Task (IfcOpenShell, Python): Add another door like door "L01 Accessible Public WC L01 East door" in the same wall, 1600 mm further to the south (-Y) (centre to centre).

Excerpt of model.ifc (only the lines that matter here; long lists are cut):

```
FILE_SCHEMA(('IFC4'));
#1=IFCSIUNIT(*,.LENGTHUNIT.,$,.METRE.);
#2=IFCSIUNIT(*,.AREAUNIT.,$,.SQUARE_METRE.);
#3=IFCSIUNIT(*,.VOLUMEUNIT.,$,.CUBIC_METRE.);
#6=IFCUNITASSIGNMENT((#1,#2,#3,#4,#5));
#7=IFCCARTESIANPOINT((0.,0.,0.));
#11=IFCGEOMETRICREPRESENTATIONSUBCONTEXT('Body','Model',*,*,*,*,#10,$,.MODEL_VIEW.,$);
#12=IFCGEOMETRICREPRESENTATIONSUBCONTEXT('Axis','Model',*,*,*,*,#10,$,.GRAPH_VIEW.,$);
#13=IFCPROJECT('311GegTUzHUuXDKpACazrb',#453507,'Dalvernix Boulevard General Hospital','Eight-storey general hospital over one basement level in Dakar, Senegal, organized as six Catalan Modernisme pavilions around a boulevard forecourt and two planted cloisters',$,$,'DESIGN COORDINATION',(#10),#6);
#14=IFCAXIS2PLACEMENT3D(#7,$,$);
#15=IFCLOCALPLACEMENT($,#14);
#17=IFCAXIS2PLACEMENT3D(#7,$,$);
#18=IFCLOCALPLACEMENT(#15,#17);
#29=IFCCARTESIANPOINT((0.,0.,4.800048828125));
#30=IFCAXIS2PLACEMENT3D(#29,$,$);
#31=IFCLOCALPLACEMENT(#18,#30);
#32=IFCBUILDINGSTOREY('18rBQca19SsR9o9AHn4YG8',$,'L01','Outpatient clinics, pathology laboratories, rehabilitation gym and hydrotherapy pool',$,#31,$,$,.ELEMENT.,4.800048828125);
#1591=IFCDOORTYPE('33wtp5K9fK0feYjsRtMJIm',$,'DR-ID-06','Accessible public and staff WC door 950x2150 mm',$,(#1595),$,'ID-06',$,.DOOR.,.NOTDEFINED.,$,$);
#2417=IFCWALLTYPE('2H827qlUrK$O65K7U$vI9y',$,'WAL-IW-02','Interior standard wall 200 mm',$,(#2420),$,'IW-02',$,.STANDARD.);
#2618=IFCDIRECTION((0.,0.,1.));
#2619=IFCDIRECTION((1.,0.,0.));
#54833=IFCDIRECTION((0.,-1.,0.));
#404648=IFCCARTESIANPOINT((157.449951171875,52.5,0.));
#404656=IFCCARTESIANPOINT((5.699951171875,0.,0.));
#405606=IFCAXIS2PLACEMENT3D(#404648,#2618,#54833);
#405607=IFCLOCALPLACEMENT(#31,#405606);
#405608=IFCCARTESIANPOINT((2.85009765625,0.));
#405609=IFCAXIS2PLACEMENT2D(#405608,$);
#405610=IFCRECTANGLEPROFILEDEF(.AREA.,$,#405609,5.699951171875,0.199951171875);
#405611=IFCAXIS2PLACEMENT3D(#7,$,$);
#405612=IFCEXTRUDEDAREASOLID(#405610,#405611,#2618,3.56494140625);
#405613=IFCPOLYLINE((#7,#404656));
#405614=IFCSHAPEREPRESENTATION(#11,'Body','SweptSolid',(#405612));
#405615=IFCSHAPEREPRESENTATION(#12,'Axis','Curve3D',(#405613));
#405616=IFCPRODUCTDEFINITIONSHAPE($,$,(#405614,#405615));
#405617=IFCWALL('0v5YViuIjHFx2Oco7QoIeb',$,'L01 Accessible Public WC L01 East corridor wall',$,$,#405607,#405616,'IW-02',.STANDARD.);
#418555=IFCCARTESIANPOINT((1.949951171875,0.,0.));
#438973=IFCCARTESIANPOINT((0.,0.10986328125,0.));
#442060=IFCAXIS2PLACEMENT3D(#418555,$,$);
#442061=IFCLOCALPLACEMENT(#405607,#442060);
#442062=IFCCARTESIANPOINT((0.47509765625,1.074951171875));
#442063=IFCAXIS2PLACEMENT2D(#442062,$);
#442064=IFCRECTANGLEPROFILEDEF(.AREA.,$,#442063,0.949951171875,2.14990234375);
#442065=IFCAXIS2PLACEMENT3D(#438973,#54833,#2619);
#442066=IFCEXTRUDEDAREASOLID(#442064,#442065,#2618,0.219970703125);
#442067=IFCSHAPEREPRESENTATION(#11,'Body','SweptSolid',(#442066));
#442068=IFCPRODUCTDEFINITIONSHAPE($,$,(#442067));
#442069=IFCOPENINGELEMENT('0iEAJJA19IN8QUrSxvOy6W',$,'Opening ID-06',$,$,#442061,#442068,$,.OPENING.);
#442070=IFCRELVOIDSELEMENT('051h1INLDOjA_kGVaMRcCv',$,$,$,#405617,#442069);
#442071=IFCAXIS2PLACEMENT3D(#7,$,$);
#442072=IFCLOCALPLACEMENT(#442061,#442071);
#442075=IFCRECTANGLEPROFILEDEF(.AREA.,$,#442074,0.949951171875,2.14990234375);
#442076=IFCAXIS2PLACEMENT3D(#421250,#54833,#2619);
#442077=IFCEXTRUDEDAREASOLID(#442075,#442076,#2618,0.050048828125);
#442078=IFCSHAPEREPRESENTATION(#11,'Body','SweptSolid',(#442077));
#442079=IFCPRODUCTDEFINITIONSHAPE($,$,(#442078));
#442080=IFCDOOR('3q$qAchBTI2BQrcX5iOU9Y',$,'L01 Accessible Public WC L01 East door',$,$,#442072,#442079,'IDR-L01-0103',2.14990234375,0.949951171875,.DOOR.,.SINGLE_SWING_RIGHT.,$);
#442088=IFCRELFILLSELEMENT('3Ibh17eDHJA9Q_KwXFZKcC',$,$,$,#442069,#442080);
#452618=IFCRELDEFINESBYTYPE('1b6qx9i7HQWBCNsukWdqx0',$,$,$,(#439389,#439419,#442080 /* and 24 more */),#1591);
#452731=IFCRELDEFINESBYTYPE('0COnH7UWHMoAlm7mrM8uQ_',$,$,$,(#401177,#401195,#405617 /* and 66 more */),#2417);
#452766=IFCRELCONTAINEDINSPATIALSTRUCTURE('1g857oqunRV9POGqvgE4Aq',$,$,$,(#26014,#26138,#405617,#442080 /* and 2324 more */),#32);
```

```python
import ifcopenshell
import ifcopenshell.api.feature
import ifcopenshell.api.geometry
import ifcopenshell.api.root
import ifcopenshell.geom
import ifcopenshell.util.element
import ifcopenshell.util.placement
import ifcopenshell.util.shape

model = ifcopenshell.open("model.ifc")
settings = ifcopenshell.geom.settings()


def volume(element):
    """Net volume in cubic metres, openings subtracted."""
    shape = ifcopenshell.geom.create_shape(settings, element)
    return ifcopenshell.util.shape.get_volume(shape.geometry)


door = model.by_guid("3q$qAchBTI2BQrcX5iOU9Y")
opening = door.FillsVoids[0].RelatingOpeningElement
wall = opening.VoidsElements[0].RelatingBuildingElement
before = volume(wall)
shift = ifcopenshell.util.placement.get_local_placement(wall.ObjectPlacement)[:3, 0] * 1.6

# copy_class copies the void relationship, type, container and properties, but no geometry.
new_opening = ifcopenshell.api.root.copy_class(model, product=opening)
new_opening.Representation = ifcopenshell.util.element.copy_deep(
    model, opening.Representation, exclude=["IfcGeometricRepresentationContext", "IfcRepresentationMap"]
)
new_door = ifcopenshell.api.root.copy_class(model, product=door)
new_door.Representation = ifcopenshell.util.element.copy_deep(
    model, door.Representation, exclude=["IfcGeometricRepresentationContext", "IfcRepresentationMap"]
)
new_door.Tag = None
ifcopenshell.api.feature.add_filling(model, opening=new_opening, element=new_door)

for old, new in ((opening, new_opening), (door, new_door)):
    matrix = ifcopenshell.util.placement.get_local_placement(old.ObjectPlacement)
    matrix[:3, 3] += shift
    ifcopenshell.api.geometry.edit_object_placement(model, product=new, matrix=matrix, is_si=False)

after = volume(wall)

print(f"wall volume {before:.3f} -> {after:.3f} m3")

model.write("model_updated.ifc")
```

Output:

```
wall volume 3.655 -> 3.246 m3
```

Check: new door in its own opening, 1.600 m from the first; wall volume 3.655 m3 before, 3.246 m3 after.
